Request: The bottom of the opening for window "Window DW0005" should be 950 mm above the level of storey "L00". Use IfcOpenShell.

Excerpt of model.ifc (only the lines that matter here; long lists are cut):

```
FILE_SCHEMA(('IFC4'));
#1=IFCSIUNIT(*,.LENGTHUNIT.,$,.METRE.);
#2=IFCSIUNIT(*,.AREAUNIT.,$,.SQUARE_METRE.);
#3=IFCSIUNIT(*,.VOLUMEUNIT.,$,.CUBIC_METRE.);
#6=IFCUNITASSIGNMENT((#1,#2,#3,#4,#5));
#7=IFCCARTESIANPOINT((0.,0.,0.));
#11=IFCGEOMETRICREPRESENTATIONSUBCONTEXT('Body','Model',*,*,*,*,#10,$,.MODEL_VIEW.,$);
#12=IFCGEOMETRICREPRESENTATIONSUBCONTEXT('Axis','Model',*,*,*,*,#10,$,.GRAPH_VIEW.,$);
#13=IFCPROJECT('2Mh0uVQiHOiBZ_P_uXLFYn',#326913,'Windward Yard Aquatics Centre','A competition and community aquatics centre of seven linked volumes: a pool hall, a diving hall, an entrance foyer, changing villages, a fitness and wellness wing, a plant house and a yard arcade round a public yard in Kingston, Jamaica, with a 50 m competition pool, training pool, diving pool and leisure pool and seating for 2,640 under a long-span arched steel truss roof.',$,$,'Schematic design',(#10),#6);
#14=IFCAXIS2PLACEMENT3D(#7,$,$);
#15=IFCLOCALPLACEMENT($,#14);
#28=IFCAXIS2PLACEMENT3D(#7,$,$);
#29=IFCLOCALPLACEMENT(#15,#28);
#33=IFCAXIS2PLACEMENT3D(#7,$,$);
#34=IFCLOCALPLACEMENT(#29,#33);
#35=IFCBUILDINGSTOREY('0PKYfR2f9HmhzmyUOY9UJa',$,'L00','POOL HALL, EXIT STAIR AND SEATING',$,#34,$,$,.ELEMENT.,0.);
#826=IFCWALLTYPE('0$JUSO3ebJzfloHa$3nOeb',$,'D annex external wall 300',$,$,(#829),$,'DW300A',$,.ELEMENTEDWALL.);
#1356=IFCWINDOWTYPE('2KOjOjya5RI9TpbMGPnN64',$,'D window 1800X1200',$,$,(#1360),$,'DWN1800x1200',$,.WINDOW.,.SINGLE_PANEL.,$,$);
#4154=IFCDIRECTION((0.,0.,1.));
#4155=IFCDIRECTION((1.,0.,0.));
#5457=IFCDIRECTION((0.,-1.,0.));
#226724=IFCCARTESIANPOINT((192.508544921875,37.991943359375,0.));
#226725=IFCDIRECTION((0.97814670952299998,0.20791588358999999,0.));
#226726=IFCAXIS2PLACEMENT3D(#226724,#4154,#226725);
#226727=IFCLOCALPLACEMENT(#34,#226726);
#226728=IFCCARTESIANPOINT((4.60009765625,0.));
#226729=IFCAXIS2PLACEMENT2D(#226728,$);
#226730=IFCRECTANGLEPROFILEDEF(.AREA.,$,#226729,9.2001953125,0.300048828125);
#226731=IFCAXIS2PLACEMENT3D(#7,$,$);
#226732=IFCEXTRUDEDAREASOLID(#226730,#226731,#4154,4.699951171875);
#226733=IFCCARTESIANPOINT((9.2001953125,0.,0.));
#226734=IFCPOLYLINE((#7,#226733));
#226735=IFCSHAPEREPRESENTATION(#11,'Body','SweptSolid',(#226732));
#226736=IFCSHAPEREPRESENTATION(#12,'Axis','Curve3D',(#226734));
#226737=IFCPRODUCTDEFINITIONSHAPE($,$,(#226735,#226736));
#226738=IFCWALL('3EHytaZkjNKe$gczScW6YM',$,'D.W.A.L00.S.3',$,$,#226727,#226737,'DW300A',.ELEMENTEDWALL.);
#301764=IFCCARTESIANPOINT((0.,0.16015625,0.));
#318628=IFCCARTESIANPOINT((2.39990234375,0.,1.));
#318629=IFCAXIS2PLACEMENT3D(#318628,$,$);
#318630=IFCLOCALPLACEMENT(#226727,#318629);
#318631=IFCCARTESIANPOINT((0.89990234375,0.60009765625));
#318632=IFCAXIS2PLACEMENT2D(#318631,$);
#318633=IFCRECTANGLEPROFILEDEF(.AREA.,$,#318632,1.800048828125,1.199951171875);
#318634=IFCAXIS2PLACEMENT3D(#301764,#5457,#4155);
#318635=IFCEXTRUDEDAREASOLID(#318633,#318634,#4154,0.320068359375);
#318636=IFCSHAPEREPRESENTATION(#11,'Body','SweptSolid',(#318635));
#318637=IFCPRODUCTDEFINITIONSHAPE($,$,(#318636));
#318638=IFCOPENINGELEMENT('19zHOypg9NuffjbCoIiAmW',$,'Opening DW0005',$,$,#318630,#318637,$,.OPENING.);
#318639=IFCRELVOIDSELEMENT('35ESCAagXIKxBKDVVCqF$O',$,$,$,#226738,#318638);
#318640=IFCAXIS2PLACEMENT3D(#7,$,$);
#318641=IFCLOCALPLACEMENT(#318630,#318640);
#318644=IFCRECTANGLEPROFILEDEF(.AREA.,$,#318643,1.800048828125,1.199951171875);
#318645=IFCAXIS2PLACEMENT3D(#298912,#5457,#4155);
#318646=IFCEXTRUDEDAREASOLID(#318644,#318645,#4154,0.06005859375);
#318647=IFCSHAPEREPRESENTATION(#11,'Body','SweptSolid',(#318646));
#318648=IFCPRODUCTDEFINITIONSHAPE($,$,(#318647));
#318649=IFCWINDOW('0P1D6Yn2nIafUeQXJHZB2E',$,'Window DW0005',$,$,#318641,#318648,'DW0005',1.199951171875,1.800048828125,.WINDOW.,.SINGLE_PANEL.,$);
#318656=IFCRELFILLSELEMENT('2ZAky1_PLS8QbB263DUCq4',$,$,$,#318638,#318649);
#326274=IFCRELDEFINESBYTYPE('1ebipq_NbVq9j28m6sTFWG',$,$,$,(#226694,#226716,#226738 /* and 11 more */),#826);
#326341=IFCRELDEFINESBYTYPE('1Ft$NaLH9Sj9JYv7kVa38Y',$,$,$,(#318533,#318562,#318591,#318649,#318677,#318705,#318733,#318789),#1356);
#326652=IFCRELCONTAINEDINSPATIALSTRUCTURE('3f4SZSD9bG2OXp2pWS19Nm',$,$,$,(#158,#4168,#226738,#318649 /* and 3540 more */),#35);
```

```python
import numpy as np
import ifcopenshell
import ifcopenshell.api.geometry
import ifcopenshell.geom
import ifcopenshell.util.element
import ifcopenshell.util.placement
import ifcopenshell.util.shape
import ifcopenshell.util.unit

model = ifcopenshell.open("model.ifc")
unit_scale = ifcopenshell.util.unit.calculate_unit_scale(model)

window = model.by_id(318649)
opening = window.FillsVoids[0].RelatingOpeningElement
storey = ifcopenshell.util.element.get_container(window, ifc_class="IfcBuildingStorey")
level = ifcopenshell.util.placement.get_local_placement(storey.ObjectPlacement)[2, 3]

# The opening's origin need not be at the sill, so measure its lowest point.
shape = ifcopenshell.geom.create_shape(ifcopenshell.geom.settings(), opening)
bottom = ifcopenshell.util.shape.get_shape_bottom_elevation(shape, shape.geometry) / unit_scale
dz = level + 0.95 / unit_scale - bottom

shift = np.array([0.0, 0.0, dz])
# The window is placed relative to its opening, so it follows when the opening moves.
matrix = ifcopenshell.util.placement.get_local_placement(opening.ObjectPlacement)
matrix[:3, 3] += shift
ifcopenshell.api.geometry.edit_object_placement(
    model, product=opening, matrix=matrix, is_si=False, should_transform_children=True
)

print(f"moved by {dz * unit_scale:+.3f} m")

model.write("model_edited.ifc")
```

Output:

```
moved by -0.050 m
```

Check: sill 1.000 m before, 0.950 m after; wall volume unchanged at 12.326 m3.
